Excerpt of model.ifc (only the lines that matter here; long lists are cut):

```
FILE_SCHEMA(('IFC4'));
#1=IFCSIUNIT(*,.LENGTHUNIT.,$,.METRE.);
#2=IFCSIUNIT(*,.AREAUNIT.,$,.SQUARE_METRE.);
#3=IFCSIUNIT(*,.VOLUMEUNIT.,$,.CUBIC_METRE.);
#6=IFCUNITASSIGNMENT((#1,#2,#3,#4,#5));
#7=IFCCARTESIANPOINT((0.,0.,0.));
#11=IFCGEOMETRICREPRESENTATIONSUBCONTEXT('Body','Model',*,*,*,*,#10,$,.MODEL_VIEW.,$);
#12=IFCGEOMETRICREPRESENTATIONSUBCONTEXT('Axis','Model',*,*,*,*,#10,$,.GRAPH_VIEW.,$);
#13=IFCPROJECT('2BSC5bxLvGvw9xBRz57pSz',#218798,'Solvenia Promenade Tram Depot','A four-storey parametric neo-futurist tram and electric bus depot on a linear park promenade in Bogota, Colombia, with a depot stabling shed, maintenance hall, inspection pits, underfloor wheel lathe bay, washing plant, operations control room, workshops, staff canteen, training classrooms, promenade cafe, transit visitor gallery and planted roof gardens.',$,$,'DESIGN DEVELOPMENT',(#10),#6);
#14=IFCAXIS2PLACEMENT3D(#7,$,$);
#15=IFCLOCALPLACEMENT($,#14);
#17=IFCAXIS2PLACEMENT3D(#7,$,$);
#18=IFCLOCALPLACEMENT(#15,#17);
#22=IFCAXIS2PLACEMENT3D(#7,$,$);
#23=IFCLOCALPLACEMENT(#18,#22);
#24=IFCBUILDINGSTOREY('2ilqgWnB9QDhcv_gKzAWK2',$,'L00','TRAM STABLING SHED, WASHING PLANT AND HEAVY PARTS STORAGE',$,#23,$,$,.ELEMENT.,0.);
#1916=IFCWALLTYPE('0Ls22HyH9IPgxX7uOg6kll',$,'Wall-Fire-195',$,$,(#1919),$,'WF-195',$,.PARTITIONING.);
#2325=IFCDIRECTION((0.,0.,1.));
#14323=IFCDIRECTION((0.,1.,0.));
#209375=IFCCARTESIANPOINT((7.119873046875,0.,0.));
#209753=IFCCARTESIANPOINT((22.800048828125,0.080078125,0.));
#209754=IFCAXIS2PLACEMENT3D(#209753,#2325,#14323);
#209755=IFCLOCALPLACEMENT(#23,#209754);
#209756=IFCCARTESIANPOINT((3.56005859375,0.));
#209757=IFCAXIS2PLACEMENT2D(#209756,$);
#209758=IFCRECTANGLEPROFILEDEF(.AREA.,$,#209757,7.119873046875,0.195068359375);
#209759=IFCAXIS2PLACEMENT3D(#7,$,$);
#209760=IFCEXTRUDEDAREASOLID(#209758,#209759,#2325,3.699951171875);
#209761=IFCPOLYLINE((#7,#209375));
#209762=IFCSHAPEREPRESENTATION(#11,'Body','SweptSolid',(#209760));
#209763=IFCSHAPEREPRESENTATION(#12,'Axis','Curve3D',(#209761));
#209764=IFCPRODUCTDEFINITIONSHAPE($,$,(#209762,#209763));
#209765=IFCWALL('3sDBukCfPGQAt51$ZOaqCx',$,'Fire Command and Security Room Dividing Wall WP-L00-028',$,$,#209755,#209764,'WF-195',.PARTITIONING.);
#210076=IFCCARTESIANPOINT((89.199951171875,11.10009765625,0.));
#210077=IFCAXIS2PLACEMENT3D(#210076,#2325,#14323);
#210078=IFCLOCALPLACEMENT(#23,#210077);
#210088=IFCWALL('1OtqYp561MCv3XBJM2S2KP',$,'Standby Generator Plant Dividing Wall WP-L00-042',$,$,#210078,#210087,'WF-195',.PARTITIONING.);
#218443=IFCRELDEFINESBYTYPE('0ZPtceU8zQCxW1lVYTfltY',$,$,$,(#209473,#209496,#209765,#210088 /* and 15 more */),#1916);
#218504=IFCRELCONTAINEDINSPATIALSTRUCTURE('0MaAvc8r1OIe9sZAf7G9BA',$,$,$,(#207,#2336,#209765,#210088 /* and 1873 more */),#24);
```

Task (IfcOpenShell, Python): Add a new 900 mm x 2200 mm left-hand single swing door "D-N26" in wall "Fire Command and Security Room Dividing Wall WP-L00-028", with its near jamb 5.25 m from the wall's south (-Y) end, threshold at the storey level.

```python
import numpy as np
import ifcopenshell
import ifcopenshell.api.feature
import ifcopenshell.api.geometry
import ifcopenshell.api.root
import ifcopenshell.api.spatial
import ifcopenshell.geom
import ifcopenshell.util.element
import ifcopenshell.util.placement
import ifcopenshell.util.representation
import ifcopenshell.util.shape
import ifcopenshell.util.unit

model = ifcopenshell.open("model.ifc")
unit_scale = ifcopenshell.util.unit.calculate_unit_scale(model)
settings = ifcopenshell.geom.settings()


def volume(element):
    """Net volume in cubic metres, openings subtracted."""
    shape = ifcopenshell.geom.create_shape(settings, element)
    return ifcopenshell.util.shape.get_volume(shape.geometry)


wall = model.by_guid("3sDBukCfPGQAt51$ZOaqCx")
storey = ifcopenshell.util.element.get_container(wall, ifc_class="IfcBuildingStorey")
context = ifcopenshell.util.representation.get_context(model, "Model", "Body", "MODEL_VIEW")
before = volume(wall)

width, height, from_end, sill = 0.9, 2.2, 5.25, 0.0  # metres

# The wall runs along its own X axis, and the end named is its -X end.
wall_shape = ifcopenshell.geom.create_shape(settings, wall)
x, y, z = ifcopenshell.util.shape.get_vertices(wall_shape.geometry).T
start = x.min() + from_end
face, thickness = float(y.min()), float(y.max() - y.min())
wall_matrix = ifcopenshell.util.placement.get_local_placement(wall.ObjectPlacement)
level = ifcopenshell.util.placement.get_local_placement(storey.ObjectPlacement)[2, 3]


def in_wall(x, y):
    """Placement at x, y metres in the wall's axes, at sill height."""
    matrix = wall_matrix.copy()
    matrix[:, 3] = wall_matrix @ np.array([x / unit_scale, y / unit_scale, 0.0, 1.0])
    matrix[2, 3] = level + sill / unit_scale
    return matrix


# Opening: a box that overshoots both wall faces by 50 mm.
opening = ifcopenshell.api.root.create_entity(model, ifc_class="IfcOpeningElement", predefined_type="OPENING")
box = ifcopenshell.api.geometry.add_wall_representation(
    model, context=context, length=width, height=height, thickness=thickness + 0.1
)
ifcopenshell.api.geometry.assign_representation(model, product=opening, representation=box)
ifcopenshell.api.geometry.edit_object_placement(model, product=opening, matrix=in_wall(start, face - 0.05), is_si=False)
ifcopenshell.api.feature.add_feature(model, feature=opening, element=wall)

door = ifcopenshell.api.root.create_entity(model, ifc_class="IfcDoor", name="D-N26", predefined_type="DOOR")
door.OverallWidth, door.OverallHeight = width / unit_scale, height / unit_scale
door.OperationType = "SINGLE_SWING_LEFT"
body = ifcopenshell.api.geometry.add_door_representation(
    model,
    context=context,
    overall_width=door.OverallWidth,
    overall_height=door.OverallHeight,
    operation_type="SINGLE_SWING_LEFT",
    lining_properties={"LiningDepth": thickness / unit_scale, "ThresholdDepth": thickness / unit_scale},
)
ifcopenshell.api.geometry.assign_representation(model, product=door, representation=body)
ifcopenshell.api.spatial.assign_container(model, products=[door], relating_structure=storey)
ifcopenshell.api.feature.add_filling(model, opening=opening, element=door)

# The lining spans the wall, so the door starts at the wall face.
ifcopenshell.api.geometry.edit_object_placement(model, product=door, matrix=in_wall(start, face), is_si=False)

after = volume(wall)

print(f"wall volume {before:.3f} -> {after:.3f} m3")

model.write("model-out.ifc")
```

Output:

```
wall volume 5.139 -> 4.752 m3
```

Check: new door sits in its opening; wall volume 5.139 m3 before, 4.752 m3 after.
